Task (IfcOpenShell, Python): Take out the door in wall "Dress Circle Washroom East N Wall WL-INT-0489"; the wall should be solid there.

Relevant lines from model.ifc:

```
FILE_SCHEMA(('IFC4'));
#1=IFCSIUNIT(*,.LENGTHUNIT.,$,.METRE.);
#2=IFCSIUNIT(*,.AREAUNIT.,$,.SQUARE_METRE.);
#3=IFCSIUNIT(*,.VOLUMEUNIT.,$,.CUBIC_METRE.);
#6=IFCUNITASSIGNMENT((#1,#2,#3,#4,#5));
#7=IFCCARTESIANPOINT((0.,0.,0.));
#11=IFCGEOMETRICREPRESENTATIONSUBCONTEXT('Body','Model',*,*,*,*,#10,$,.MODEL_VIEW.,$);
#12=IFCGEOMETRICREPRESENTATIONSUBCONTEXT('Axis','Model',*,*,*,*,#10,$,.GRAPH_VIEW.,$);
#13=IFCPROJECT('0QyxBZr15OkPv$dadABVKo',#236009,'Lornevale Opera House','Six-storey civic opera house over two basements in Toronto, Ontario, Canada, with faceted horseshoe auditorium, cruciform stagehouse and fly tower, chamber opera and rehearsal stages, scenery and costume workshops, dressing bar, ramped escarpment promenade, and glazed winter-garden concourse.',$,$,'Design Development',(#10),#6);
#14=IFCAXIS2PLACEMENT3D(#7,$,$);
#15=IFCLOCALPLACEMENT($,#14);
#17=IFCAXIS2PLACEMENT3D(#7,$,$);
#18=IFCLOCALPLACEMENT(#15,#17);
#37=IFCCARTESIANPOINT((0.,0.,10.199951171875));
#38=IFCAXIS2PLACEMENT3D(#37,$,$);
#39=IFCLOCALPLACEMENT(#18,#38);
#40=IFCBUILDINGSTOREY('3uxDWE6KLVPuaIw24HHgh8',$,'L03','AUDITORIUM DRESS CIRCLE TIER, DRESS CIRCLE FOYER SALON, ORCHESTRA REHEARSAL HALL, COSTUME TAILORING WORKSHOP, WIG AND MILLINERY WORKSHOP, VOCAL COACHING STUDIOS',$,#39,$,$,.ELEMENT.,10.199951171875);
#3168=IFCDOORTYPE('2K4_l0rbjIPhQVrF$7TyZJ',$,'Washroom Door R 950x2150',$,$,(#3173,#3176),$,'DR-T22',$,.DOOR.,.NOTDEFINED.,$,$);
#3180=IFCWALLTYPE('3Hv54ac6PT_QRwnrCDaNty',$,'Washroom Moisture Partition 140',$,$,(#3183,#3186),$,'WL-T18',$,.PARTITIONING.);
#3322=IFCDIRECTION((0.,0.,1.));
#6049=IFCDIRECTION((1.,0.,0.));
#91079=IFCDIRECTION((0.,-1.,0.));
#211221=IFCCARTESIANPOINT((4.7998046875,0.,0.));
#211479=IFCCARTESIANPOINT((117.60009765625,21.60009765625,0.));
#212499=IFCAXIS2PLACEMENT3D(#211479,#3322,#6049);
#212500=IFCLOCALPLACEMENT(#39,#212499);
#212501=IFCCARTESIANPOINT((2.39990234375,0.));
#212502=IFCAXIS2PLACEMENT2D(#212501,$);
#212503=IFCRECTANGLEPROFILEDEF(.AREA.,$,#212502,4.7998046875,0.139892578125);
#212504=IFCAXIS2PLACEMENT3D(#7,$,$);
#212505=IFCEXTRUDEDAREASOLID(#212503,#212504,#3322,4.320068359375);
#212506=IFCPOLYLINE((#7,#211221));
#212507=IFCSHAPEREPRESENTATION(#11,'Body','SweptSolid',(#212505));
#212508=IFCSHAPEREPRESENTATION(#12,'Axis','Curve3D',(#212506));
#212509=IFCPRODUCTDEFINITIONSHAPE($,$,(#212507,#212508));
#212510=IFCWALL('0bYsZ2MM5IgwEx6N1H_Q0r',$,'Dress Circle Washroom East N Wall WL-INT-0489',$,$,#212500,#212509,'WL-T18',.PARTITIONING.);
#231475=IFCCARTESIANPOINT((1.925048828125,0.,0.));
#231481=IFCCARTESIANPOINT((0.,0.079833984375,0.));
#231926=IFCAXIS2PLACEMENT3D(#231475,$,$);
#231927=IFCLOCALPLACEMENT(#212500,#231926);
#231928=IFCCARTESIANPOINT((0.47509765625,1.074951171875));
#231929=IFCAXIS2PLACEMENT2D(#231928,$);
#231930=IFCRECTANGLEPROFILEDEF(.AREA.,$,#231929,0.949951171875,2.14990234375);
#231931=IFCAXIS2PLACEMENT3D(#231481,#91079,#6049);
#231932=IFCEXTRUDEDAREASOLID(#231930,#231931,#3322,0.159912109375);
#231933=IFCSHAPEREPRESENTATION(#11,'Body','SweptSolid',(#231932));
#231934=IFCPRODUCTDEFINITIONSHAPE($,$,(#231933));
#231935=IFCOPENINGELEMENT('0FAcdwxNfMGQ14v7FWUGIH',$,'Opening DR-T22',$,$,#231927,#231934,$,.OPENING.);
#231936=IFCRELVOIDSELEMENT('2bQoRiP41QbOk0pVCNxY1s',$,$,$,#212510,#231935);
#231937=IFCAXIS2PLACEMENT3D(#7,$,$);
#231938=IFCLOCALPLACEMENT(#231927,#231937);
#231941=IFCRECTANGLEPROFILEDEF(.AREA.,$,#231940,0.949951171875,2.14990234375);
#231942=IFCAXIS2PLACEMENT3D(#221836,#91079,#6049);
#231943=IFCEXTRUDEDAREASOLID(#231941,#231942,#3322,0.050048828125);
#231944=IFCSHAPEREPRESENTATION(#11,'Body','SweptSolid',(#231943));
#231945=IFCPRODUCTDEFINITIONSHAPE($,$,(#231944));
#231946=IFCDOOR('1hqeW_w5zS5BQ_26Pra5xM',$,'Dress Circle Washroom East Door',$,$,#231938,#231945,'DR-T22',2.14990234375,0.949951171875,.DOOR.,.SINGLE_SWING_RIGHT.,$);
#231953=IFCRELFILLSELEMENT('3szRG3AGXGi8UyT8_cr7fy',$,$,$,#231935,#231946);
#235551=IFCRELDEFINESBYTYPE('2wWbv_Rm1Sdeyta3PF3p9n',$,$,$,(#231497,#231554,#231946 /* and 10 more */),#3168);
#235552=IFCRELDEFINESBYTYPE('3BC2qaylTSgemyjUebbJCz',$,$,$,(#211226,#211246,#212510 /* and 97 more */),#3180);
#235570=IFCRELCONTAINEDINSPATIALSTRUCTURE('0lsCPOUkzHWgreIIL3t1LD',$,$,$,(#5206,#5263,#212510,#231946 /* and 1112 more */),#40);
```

```python
import ifcopenshell
import ifcopenshell.api.feature
import ifcopenshell.api.root
import ifcopenshell.geom
import ifcopenshell.util.shape

model = ifcopenshell.open("model.ifc")
settings = ifcopenshell.geom.settings()


def volume(element):
    """Net volume in cubic metres, openings subtracted."""
    shape = ifcopenshell.geom.create_shape(settings, element)
    return ifcopenshell.util.shape.get_volume(shape.geometry)


door = model.by_id(231946)
opening = door.FillsVoids[0].RelatingOpeningElement
wall = opening.VoidsElements[0].RelatingBuildingElement
before = volume(wall)

ifcopenshell.api.root.remove_product(model, product=door)
ifcopenshell.api.feature.remove_feature(model, feature=opening)

after = volume(wall)

print(f"wall volume {before:.3f} -> {after:.3f} m3")

model.write("model-out.ifc")
```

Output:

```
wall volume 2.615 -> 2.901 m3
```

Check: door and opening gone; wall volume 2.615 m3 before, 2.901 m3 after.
